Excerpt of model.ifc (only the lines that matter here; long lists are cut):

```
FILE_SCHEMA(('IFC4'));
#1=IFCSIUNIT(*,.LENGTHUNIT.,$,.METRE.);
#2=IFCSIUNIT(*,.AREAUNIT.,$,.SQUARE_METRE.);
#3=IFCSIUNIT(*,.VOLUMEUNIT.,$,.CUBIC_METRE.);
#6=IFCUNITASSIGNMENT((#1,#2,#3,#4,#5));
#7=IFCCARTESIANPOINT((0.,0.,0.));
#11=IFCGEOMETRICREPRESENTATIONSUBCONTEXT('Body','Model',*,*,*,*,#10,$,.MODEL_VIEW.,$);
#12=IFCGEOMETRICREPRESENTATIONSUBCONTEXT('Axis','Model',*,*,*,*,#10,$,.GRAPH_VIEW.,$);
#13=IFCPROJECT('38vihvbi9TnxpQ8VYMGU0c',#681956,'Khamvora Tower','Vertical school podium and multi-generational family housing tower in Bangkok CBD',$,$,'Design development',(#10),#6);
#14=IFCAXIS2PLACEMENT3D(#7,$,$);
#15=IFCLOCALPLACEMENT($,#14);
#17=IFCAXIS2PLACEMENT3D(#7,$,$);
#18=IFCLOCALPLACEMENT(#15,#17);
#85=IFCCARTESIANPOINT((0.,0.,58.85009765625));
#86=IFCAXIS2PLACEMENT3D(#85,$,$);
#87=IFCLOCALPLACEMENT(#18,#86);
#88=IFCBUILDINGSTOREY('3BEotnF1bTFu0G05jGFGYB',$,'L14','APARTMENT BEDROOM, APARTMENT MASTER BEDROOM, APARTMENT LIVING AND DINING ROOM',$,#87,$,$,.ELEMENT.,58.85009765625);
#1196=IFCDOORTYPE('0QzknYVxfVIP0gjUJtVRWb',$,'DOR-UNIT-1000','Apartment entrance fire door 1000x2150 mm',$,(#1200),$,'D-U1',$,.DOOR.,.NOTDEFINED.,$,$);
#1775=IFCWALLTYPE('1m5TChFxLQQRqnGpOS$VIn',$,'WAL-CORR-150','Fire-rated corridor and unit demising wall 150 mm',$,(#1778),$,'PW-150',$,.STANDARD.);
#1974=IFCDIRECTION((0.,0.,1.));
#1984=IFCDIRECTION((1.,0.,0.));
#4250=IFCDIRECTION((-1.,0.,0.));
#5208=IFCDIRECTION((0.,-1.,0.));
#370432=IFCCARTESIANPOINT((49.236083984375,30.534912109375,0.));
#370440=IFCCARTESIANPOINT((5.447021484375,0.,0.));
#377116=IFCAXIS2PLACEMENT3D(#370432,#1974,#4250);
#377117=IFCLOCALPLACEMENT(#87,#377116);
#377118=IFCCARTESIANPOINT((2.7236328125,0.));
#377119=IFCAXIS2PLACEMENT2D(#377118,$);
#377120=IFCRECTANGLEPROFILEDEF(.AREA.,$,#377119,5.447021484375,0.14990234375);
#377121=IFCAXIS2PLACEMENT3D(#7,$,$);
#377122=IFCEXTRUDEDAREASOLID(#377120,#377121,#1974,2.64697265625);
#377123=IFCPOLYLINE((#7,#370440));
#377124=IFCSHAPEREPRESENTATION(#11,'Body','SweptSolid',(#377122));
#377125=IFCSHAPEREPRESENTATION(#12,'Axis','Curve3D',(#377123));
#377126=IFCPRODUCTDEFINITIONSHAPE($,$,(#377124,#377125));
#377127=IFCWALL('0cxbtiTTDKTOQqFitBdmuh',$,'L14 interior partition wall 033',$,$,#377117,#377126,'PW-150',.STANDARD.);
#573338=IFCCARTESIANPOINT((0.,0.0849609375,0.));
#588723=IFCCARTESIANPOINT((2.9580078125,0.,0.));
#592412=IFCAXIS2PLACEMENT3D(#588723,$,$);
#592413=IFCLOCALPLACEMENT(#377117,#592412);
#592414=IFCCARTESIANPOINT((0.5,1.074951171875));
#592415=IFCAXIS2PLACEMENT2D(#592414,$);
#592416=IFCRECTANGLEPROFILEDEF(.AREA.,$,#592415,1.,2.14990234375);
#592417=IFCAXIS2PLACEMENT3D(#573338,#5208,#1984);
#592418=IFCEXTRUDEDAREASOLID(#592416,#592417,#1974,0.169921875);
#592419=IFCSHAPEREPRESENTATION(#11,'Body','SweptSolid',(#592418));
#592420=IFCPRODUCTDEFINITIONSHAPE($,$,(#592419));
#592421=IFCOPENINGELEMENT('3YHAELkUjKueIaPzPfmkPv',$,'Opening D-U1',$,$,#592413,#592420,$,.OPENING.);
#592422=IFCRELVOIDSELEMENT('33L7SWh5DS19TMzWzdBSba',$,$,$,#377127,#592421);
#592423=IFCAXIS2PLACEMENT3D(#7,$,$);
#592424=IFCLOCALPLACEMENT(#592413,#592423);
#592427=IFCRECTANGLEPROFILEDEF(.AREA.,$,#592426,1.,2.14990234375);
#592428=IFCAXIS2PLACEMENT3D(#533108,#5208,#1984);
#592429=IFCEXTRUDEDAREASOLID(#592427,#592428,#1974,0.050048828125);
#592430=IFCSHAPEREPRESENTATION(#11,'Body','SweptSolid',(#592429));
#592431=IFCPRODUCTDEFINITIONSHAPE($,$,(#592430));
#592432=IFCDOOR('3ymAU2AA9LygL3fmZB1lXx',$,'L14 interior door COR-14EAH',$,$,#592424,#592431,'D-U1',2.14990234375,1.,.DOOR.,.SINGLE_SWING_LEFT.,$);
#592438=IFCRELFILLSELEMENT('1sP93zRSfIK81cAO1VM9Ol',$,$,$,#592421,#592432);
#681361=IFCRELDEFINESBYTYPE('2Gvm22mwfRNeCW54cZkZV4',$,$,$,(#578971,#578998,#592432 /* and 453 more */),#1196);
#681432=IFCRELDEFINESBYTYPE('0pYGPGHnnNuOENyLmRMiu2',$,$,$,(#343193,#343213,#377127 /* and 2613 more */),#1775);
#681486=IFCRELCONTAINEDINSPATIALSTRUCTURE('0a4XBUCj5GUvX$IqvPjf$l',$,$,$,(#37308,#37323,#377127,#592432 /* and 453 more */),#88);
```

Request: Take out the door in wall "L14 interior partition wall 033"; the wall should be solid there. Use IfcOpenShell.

```python
import ifcopenshell
import ifcopenshell.api.feature
import ifcopenshell.api.root
import ifcopenshell.geom
import ifcopenshell.util.shape

model = ifcopenshell.open("model.ifc")
settings = ifcopenshell.geom.settings()


def volume(element):
    """Net volume in cubic metres, openings subtracted."""
    shape = ifcopenshell.geom.create_shape(settings, element)
    return ifcopenshell.util.shape.get_volume(shape.geometry)


door = model.by_guid("3ymAU2AA9LygL3fmZB1lXx")
opening = door.FillsVoids[0].RelatingOpeningElement
wall = opening.VoidsElements[0].RelatingBuildingElement
before = volume(wall)

ifcopenshell.api.root.remove_product(model, product=door)
ifcopenshell.api.feature.remove_feature(model, feature=opening)

after = volume(wall)

print(f"wall volume {before:.3f} -> {after:.3f} m3")

model.write("model-out.ifc")
```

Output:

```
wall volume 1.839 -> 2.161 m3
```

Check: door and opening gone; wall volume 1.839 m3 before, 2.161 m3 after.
